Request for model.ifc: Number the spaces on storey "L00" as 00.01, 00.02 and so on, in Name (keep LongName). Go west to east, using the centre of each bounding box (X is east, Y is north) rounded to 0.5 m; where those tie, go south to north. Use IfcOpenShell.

First a look at what the model holds.

```python
import ifcopenshell
import ifcopenshell.util.element
import ifcopenshell.util.placement

model = ifcopenshell.open("model.ifc")
print(model.schema)
storey = next(s for s in model.by_type("IfcBuildingStorey") if s.Name == "L00")
spaces = [e for e in ifcopenshell.util.element.get_decomposition(storey) if e.is_a("IfcSpace")]
for e in sorted(spaces, key=lambda e: e.id()):
    origin = ifcopenshell.util.placement.get_local_placement(e.ObjectPlacement)[:3, 3]
    print(e.id(), e.Name, e.LongName, origin.round(2) + 0.0, sep=" | ")
```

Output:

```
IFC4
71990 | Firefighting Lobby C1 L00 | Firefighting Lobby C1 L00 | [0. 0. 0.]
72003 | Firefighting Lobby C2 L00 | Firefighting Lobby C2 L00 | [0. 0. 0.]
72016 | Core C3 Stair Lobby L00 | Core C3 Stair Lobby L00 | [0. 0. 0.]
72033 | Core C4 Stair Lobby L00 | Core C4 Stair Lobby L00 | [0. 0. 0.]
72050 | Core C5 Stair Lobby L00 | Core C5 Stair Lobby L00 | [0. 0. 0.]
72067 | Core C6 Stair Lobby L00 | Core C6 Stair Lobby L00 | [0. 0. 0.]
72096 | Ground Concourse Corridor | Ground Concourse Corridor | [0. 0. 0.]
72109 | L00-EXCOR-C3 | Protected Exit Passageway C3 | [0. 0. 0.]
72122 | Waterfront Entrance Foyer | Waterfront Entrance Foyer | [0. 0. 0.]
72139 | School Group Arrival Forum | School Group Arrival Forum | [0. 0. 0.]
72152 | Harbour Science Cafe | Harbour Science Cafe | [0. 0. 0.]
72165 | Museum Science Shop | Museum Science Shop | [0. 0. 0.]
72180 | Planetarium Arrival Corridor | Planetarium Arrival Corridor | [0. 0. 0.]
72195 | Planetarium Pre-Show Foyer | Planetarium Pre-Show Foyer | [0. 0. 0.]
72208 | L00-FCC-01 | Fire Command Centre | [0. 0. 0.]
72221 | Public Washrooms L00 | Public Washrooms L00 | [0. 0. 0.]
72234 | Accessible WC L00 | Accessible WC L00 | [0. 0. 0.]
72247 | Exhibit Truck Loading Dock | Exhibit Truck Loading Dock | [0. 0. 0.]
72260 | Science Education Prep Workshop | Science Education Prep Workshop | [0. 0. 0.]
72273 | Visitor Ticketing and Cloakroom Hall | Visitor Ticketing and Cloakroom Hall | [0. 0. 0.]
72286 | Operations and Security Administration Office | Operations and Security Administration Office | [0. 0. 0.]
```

```python
import ifcopenshell
import ifcopenshell.geom
import ifcopenshell.util.element
import ifcopenshell.util.shape

model = ifcopenshell.open("model.ifc")
settings = ifcopenshell.geom.settings()
settings.set("use-world-coords", True)


def centre(element):
    shape = ifcopenshell.geom.create_shape(settings, element)
    return ifcopenshell.util.shape.get_bbox_centroid(shape.geometry)


storey = next(s for s in model.by_type("IfcBuildingStorey") if s.Name == "L00")
spaces = [e for e in ifcopenshell.util.element.get_decomposition(storey) if e.is_a("IfcSpace")]

# Insertion points can sit at a corner or the storey origin, so sort by the geometry (in metres).
centres = {e: centre(e) for e in spaces}
spaces.sort(key=lambda e: (round(centres[e][0] / 0.5), centres[e][1]))

for i, e in enumerate(spaces, start=1):
    number = f"00.{i:02d}"
    e.Name = number
    print(e.id(), number)

model.write("model_rev.ifc")
```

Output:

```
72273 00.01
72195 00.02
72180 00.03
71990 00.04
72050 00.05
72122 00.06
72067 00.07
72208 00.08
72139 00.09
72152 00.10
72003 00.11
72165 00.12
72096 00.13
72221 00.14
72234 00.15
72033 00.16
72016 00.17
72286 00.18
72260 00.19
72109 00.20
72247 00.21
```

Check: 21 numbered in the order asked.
